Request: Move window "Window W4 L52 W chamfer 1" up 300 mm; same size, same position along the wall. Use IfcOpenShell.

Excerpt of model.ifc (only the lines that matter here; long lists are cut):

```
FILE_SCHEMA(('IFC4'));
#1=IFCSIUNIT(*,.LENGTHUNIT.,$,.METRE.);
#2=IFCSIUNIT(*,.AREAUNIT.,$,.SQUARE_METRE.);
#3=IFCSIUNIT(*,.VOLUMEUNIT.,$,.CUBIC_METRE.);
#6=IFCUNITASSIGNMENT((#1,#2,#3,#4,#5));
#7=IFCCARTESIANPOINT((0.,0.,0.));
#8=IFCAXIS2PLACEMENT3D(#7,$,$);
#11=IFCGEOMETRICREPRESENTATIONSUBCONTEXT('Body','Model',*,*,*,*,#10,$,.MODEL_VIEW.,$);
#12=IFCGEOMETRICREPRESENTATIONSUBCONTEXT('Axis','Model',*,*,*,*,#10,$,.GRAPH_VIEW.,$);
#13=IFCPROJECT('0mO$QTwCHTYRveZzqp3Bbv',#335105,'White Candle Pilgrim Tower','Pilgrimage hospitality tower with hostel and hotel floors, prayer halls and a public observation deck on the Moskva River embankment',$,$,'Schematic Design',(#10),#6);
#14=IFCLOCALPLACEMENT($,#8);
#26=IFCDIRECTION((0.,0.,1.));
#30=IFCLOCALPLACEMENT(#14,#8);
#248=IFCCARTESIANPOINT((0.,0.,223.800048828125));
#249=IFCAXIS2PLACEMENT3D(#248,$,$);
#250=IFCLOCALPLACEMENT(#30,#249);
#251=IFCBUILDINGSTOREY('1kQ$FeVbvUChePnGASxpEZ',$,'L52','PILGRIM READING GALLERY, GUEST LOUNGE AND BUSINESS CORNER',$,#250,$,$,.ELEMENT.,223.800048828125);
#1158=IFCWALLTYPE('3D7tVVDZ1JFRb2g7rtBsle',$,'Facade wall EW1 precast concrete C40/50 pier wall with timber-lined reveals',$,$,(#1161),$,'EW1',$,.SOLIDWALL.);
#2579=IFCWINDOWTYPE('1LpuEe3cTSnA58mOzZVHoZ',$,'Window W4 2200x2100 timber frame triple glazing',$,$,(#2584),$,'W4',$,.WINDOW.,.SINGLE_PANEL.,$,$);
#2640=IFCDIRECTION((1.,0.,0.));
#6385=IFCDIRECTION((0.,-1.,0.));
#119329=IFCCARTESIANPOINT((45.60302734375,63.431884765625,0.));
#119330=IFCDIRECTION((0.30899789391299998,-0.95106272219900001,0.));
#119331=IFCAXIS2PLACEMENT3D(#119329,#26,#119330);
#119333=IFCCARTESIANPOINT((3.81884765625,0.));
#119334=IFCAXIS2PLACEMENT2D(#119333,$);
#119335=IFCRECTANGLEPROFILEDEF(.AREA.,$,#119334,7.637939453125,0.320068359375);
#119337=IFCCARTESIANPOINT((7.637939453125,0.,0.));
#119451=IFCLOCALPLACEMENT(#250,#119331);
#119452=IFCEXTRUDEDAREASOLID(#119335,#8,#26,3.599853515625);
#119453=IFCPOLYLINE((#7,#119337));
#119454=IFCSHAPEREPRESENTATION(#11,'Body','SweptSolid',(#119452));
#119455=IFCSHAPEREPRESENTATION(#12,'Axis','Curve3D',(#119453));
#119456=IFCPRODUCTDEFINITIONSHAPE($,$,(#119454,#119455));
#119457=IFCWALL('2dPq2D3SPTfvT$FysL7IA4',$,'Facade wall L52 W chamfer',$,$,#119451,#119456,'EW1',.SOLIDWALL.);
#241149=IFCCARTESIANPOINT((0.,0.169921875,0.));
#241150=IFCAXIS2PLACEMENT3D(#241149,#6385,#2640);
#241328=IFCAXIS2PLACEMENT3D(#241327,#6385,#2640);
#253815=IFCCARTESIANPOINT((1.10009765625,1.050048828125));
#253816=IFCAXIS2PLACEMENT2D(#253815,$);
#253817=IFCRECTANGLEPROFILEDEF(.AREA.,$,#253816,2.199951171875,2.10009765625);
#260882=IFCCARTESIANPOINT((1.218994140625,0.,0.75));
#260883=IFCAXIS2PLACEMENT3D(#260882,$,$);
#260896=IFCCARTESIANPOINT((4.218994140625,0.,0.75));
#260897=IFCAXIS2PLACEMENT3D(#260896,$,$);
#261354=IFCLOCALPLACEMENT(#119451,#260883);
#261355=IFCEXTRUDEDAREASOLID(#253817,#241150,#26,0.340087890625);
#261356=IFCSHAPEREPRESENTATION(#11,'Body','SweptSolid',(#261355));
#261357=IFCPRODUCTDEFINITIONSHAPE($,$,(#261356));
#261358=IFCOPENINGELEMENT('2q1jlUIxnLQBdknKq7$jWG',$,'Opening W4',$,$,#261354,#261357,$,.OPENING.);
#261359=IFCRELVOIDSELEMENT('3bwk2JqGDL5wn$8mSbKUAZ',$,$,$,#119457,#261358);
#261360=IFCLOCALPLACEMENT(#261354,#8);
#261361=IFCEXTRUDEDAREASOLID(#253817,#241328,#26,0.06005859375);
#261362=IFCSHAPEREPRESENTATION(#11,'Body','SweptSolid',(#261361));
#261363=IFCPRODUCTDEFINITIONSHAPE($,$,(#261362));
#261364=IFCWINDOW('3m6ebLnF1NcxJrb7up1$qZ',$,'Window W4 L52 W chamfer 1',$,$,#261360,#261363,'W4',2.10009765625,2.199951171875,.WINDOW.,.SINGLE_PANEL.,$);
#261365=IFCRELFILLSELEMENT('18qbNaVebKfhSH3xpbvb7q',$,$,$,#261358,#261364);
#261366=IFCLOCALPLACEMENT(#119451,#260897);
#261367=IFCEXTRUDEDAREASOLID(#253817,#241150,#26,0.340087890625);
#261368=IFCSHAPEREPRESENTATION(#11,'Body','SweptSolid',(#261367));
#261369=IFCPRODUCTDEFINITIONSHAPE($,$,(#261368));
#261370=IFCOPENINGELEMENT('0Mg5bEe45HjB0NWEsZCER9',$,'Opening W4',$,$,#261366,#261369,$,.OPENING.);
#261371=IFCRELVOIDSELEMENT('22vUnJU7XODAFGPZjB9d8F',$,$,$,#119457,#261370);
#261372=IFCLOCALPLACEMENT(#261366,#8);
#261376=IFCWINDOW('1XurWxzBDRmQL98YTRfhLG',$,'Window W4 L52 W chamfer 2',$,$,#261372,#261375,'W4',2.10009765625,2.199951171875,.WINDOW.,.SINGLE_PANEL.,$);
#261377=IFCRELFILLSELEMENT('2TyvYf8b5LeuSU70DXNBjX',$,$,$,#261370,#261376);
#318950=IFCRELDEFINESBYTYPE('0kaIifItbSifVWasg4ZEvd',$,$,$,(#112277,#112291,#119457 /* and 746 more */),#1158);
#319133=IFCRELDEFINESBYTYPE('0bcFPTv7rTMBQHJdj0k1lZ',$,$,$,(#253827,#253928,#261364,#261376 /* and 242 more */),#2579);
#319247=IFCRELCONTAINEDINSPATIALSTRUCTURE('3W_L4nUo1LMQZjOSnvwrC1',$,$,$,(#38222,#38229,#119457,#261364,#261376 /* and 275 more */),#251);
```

```python
import numpy as np
import ifcopenshell
import ifcopenshell.api.geometry
import ifcopenshell.util.placement
import ifcopenshell.util.unit

model = ifcopenshell.open("model.ifc")
unit_scale = ifcopenshell.util.unit.calculate_unit_scale(model)

window = model.by_guid("3m6ebLnF1NcxJrb7up1$qZ")
opening = window.FillsVoids[0].RelatingOpeningElement
dz = 0.3 / unit_scale

shift = np.array([0.0, 0.0, dz])
# The window is placed relative to its opening, so it follows when the opening moves.
matrix = ifcopenshell.util.placement.get_local_placement(opening.ObjectPlacement)
matrix[:3, 3] += shift
ifcopenshell.api.geometry.edit_object_placement(
    model, product=opening, matrix=matrix, is_si=False, should_transform_children=True
)

print(f"moved by {dz * unit_scale:+.3f} m")

model.write("model-out.ifc")
```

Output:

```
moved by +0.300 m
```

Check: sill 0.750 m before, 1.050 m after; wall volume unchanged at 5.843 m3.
